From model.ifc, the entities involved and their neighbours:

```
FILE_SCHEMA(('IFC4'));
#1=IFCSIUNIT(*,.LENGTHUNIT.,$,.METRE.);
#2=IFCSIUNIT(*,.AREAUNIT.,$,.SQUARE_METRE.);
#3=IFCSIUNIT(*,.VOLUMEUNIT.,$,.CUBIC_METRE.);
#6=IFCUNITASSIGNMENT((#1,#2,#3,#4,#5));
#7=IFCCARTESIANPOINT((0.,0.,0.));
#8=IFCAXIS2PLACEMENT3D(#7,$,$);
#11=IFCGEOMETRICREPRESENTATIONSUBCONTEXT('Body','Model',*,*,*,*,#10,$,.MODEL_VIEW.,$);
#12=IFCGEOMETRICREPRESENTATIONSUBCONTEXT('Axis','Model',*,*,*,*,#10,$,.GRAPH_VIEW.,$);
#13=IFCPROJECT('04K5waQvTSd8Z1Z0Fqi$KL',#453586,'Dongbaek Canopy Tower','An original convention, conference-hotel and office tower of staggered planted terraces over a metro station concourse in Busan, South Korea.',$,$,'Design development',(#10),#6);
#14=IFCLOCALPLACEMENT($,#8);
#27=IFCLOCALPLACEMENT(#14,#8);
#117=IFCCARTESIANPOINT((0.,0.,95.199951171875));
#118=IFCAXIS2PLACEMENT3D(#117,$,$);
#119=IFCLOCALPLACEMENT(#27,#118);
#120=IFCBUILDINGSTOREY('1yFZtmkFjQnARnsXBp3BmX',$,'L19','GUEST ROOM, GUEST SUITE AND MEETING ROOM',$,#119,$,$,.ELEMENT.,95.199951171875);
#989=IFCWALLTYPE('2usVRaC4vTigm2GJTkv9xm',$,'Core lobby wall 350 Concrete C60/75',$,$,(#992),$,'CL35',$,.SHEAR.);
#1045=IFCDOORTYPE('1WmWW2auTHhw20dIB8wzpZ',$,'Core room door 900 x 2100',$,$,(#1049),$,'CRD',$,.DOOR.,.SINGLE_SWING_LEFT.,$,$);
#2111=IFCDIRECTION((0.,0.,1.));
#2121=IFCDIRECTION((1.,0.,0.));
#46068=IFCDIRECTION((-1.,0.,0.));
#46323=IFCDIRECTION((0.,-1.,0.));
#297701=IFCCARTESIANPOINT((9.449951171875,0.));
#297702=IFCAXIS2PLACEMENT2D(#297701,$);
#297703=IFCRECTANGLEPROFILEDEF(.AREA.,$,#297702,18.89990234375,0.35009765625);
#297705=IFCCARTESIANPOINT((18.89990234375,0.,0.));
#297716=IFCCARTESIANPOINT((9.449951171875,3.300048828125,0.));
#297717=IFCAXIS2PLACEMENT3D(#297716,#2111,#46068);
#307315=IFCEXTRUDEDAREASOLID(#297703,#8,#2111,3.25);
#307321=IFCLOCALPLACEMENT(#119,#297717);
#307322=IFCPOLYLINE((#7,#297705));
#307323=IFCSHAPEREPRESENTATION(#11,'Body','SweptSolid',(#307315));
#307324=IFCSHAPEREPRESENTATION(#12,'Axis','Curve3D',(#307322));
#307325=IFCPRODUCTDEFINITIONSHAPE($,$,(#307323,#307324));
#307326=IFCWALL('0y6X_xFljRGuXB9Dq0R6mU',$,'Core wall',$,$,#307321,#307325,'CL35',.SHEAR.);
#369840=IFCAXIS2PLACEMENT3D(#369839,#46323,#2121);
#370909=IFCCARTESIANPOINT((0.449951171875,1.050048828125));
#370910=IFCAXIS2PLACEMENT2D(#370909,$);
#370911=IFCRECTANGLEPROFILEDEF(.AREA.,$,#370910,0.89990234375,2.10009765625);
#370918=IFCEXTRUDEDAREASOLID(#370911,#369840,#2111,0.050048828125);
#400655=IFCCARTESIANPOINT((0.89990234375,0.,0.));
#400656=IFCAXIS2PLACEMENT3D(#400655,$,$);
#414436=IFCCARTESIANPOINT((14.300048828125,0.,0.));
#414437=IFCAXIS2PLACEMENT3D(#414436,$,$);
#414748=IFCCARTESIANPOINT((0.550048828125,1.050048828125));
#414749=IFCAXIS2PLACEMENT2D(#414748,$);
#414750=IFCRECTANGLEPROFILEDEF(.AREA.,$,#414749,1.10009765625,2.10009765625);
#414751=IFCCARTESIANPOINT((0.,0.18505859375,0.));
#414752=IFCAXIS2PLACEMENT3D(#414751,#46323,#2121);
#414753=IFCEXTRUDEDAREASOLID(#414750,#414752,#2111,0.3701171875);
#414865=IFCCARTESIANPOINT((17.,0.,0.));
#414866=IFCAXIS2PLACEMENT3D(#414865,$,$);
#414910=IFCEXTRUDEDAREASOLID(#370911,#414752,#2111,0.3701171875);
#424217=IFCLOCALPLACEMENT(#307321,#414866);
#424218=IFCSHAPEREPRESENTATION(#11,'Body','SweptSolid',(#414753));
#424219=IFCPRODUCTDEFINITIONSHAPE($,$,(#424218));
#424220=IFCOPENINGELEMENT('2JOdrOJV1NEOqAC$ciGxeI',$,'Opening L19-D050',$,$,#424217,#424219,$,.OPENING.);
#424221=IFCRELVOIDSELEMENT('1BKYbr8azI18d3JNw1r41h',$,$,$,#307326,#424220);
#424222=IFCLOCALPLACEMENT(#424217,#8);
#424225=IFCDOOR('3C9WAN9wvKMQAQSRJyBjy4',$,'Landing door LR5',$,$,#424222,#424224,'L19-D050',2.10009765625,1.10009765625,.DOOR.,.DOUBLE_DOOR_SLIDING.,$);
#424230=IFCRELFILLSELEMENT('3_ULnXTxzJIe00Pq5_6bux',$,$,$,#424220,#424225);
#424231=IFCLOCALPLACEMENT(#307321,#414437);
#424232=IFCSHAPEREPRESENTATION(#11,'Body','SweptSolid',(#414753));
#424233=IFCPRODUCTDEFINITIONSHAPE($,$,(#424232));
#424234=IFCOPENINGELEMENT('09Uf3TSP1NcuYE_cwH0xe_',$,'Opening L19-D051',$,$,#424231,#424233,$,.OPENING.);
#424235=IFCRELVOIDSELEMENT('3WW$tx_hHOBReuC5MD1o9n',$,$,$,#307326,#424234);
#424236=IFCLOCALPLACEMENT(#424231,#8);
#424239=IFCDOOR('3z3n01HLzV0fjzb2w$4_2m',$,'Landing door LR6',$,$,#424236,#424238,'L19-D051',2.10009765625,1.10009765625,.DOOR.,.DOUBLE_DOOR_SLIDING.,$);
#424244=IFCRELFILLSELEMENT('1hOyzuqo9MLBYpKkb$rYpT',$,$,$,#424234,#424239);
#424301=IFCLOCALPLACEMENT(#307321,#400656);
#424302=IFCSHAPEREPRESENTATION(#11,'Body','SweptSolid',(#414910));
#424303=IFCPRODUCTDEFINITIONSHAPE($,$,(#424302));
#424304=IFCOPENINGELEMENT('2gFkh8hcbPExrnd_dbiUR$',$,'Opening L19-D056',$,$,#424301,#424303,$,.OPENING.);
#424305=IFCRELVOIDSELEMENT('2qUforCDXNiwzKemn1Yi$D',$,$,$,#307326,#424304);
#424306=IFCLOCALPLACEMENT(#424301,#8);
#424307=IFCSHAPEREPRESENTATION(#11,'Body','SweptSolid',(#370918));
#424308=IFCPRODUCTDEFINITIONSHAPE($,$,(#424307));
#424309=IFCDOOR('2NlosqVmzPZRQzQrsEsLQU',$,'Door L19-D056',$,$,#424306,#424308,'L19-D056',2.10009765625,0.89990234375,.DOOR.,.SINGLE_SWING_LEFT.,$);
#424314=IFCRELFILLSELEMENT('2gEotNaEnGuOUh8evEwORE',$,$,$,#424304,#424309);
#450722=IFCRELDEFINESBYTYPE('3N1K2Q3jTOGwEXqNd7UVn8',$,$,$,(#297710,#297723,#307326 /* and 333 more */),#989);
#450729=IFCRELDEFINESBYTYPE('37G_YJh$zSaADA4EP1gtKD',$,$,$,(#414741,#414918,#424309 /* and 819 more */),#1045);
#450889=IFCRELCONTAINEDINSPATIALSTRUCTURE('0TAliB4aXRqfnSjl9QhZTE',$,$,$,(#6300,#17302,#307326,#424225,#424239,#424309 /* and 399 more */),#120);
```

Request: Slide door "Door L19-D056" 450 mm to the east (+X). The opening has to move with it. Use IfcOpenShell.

```python
import ifcopenshell
import ifcopenshell.api.geometry
import ifcopenshell.util.placement

model = ifcopenshell.open("model.ifc")

door = model.by_guid("2NlosqVmzPZRQzQrsEsLQU")
opening = door.FillsVoids[0].RelatingOpeningElement
wall = opening.VoidsElements[0].RelatingBuildingElement

wall_matrix = ifcopenshell.util.placement.get_local_placement(wall.ObjectPlacement)
shift = wall_matrix[:3, 0] * -0.45
before = ifcopenshell.util.placement.get_local_placement(door.ObjectPlacement)[:3, 3].copy()

# The door is placed relative to its opening, so it follows when the opening moves.
matrix = ifcopenshell.util.placement.get_local_placement(opening.ObjectPlacement)
matrix[:3, 3] += shift
ifcopenshell.api.geometry.edit_object_placement(
    model, product=opening, matrix=matrix, is_si=False, should_transform_children=True
)

after = ifcopenshell.util.placement.get_local_placement(door.ObjectPlacement)[:3, 3]
print("door moved by", (after - before).round(3) + 0.0)

model.write("model_rev.ifc")
```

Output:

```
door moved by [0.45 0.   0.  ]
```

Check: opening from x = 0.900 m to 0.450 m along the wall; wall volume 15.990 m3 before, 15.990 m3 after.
